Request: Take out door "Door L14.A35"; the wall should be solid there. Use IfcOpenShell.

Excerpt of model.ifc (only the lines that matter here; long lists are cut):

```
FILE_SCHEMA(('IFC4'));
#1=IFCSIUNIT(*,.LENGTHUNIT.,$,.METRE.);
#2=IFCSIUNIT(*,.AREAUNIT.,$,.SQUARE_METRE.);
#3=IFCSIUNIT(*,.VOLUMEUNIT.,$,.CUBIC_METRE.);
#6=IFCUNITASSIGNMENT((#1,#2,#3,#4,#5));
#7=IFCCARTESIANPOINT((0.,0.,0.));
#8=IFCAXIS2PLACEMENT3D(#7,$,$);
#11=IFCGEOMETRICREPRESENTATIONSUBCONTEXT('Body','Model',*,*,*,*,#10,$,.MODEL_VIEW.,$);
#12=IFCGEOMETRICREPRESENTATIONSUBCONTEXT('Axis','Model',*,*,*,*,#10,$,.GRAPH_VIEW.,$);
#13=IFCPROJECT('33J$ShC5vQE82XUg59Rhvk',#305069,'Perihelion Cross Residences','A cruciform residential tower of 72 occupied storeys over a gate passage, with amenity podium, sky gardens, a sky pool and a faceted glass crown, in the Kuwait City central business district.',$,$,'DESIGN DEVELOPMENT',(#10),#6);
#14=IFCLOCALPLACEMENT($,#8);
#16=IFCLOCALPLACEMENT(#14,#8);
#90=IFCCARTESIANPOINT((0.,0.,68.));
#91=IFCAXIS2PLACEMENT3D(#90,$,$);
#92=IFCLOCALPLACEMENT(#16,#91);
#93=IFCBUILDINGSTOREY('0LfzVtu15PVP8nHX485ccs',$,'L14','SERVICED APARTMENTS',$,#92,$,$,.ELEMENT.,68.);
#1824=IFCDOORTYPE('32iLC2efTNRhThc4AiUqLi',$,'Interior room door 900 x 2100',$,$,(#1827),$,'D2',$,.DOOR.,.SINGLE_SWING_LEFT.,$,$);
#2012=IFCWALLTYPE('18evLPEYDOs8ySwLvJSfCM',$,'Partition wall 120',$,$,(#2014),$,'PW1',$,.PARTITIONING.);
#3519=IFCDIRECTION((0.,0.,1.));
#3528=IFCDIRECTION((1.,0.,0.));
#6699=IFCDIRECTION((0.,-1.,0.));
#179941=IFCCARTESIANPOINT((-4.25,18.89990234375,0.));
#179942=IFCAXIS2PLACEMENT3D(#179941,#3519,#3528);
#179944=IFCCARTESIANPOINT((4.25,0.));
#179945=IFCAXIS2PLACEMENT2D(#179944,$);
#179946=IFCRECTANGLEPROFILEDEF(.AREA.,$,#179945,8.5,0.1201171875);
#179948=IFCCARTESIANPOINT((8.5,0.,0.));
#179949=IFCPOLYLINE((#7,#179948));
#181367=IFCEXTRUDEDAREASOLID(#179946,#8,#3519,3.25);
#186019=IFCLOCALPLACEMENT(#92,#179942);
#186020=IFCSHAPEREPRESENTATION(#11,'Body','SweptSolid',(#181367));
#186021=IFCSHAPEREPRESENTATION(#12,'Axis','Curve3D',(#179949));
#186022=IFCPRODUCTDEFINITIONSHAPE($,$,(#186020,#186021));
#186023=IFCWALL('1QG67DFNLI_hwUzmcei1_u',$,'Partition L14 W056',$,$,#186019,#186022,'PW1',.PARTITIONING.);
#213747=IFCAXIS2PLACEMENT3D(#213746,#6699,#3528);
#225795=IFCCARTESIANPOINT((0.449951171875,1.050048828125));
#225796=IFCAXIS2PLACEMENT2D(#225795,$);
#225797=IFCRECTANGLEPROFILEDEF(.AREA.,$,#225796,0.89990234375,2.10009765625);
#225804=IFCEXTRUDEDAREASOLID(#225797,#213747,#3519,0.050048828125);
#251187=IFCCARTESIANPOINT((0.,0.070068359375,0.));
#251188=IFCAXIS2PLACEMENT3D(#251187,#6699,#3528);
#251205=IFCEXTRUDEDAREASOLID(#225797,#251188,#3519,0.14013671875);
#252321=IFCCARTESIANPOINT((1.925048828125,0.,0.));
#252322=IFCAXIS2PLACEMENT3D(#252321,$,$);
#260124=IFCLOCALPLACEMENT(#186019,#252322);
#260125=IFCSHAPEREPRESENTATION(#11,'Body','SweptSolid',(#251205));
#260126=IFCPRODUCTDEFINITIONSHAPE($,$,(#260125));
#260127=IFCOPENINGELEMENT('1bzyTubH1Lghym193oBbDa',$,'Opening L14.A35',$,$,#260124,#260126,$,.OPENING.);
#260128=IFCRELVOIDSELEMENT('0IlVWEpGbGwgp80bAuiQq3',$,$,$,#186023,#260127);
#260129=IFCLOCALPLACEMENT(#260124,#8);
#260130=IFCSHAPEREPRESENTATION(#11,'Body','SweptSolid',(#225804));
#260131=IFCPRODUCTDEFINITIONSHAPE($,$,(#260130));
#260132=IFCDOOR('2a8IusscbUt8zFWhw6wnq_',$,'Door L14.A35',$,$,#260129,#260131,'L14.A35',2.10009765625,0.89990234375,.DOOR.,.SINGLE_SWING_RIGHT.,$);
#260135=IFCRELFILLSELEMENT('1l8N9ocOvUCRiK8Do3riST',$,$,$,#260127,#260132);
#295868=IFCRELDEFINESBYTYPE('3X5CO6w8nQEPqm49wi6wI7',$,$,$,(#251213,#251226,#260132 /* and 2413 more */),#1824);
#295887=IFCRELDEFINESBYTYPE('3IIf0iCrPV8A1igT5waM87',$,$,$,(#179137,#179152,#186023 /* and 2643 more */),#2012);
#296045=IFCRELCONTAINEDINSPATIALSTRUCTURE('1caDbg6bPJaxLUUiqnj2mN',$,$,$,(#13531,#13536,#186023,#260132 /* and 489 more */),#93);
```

```python
import ifcopenshell
import ifcopenshell.api.feature
import ifcopenshell.api.root
import ifcopenshell.geom
import ifcopenshell.util.shape

model = ifcopenshell.open("model.ifc")
settings = ifcopenshell.geom.settings()


def volume(element):
    """Net volume in cubic metres, openings subtracted."""
    shape = ifcopenshell.geom.create_shape(settings, element)
    return ifcopenshell.util.shape.get_volume(shape.geometry)


door = model.by_guid("2a8IusscbUt8zFWhw6wnq_")
opening = door.FillsVoids[0].RelatingOpeningElement
wall = opening.VoidsElements[0].RelatingBuildingElement
before = volume(wall)

ifcopenshell.api.root.remove_product(model, product=door)
ifcopenshell.api.feature.remove_feature(model, feature=opening)

after = volume(wall)

print(f"wall volume {before:.3f} -> {after:.3f} m3")

model.write("model_edited.ifc")
```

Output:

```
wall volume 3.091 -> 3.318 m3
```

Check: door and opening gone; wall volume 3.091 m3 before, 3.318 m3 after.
